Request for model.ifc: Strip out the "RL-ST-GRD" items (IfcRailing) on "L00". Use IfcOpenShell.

First a look at what the model holds.

```python
import ifcopenshell
import ifcopenshell.util.element

model = ifcopenshell.open("model.ifc")
print(model.schema)
storey = next(s for s in model.by_type("IfcBuildingStorey") if s.Name == "L00")
railings = [e for e in ifcopenshell.util.element.get_decomposition(storey) if e.is_a("IfcRailing")]
seen = {}
for e in railings:
    element_type = ifcopenshell.util.element.get_type(e)
    name = element_type.Name if element_type not in (None, e) else None
    seen[name] = seen.get(name, 0) + 1
for name, count in sorted(seen.items(), key=str):
    print(count, "x", name)
```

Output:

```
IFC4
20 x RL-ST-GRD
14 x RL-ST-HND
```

```python
import ifcopenshell
import ifcopenshell.api.root
import ifcopenshell.util.element

model = ifcopenshell.open("model.ifc")

storey = next(s for s in model.by_type("IfcBuildingStorey") if s.Name == "L00")
railings = [e for e in ifcopenshell.util.element.get_decomposition(storey) if e.is_a("IfcRailing")]
targets = [e for e in railings if (t := ifcopenshell.util.element.get_type(e)) not in (None, e) and t.Name == "RL-ST-GRD"]

for e in targets:
    ifcopenshell.api.root.remove_product(model, product=e)
print(len(targets), "removed")

model.write("model_v2.ifc")
```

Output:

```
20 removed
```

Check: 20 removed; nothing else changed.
